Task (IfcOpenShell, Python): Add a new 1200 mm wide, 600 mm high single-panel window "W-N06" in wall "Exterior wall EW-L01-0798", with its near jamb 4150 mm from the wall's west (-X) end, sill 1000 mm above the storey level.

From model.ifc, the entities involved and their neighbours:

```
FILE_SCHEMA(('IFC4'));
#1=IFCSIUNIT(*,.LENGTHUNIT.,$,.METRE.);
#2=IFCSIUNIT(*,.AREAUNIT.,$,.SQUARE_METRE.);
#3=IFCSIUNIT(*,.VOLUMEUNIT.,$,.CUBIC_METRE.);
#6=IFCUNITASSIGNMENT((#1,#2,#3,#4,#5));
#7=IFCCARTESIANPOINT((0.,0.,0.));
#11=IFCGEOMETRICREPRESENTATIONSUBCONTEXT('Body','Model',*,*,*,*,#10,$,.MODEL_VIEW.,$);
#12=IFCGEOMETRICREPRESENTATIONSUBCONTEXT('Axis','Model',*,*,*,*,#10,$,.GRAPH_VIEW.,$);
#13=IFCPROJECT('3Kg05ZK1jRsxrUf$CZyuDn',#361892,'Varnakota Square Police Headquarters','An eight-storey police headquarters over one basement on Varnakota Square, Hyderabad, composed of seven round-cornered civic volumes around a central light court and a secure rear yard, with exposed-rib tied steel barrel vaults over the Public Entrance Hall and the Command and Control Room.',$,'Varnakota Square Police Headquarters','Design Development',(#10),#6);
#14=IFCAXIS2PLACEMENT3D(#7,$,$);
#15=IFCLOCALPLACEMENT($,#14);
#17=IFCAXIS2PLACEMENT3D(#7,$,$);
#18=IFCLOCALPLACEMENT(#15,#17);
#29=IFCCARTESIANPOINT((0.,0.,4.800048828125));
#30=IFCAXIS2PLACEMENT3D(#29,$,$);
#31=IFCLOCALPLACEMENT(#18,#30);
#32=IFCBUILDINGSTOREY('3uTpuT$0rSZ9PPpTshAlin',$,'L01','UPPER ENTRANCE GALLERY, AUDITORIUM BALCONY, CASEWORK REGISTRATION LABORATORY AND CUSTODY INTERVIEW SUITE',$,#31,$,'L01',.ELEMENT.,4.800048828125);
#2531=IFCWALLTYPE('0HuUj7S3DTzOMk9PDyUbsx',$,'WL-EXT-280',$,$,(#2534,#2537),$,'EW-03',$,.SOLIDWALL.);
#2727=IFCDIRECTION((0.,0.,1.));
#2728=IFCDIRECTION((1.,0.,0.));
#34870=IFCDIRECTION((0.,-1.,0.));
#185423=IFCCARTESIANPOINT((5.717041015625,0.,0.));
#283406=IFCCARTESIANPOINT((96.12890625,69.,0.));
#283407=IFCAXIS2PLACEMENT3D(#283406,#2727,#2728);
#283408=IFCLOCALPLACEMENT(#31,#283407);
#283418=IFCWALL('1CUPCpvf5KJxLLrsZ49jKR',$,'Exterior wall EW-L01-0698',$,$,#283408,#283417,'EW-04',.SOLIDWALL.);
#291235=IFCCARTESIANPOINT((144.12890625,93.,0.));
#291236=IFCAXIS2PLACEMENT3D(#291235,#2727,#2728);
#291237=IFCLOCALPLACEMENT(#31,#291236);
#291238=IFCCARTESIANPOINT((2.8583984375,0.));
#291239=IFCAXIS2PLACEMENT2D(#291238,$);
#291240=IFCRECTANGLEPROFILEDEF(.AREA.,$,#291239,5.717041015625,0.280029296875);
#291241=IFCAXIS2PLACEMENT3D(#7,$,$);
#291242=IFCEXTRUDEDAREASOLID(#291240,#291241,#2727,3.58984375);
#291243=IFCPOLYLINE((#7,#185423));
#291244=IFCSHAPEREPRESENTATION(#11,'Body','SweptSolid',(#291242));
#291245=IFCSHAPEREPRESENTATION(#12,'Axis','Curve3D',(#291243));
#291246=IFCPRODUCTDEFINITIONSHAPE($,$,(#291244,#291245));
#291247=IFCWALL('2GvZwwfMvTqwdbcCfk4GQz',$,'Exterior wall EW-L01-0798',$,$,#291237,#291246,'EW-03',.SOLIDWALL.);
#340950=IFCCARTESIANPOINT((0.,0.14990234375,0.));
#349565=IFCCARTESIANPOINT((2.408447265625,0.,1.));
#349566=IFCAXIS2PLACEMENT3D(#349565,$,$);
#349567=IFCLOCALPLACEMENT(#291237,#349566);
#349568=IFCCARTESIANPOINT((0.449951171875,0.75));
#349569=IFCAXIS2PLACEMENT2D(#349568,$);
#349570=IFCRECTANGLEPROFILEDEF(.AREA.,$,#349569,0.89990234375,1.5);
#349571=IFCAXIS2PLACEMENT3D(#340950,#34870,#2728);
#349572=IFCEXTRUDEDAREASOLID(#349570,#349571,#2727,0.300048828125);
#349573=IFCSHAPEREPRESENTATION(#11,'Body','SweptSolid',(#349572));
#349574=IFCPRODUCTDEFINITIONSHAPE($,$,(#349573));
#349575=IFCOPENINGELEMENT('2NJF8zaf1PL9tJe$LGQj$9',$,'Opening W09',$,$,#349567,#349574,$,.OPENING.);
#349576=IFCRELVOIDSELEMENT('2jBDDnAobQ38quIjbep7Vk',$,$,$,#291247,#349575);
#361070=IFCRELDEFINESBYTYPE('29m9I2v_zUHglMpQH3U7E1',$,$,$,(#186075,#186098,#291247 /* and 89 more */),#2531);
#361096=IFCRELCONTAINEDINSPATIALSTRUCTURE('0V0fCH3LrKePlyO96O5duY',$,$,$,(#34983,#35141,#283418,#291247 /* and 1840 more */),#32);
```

```python
import numpy as np
import ifcopenshell
import ifcopenshell.api.feature
import ifcopenshell.api.geometry
import ifcopenshell.api.root
import ifcopenshell.api.spatial
import ifcopenshell.geom
import ifcopenshell.util.element
import ifcopenshell.util.placement
import ifcopenshell.util.representation
import ifcopenshell.util.shape
import ifcopenshell.util.unit

model = ifcopenshell.open("model.ifc")
unit_scale = ifcopenshell.util.unit.calculate_unit_scale(model)
settings = ifcopenshell.geom.settings()


def volume(element):
    """Net volume in cubic metres, openings subtracted."""
    shape = ifcopenshell.geom.create_shape(settings, element)
    return ifcopenshell.util.shape.get_volume(shape.geometry)


wall = model.by_guid("2GvZwwfMvTqwdbcCfk4GQz")
storey = ifcopenshell.util.element.get_container(wall, ifc_class="IfcBuildingStorey")
context = ifcopenshell.util.representation.get_context(model, "Model", "Body", "MODEL_VIEW")
before = volume(wall)

width, height, from_end, sill = 1.2, 0.6, 4.15, 1  # metres

# The wall runs along its own X axis, and the end named is its -X end.
wall_shape = ifcopenshell.geom.create_shape(settings, wall)
x, y, z = ifcopenshell.util.shape.get_vertices(wall_shape.geometry).T
start = x.min() + from_end
face, thickness = float(y.min()), float(y.max() - y.min())
wall_matrix = ifcopenshell.util.placement.get_local_placement(wall.ObjectPlacement)
level = ifcopenshell.util.placement.get_local_placement(storey.ObjectPlacement)[2, 3]


def in_wall(x, y):
    """Placement at x, y metres in the wall's axes, at sill height."""
    matrix = wall_matrix.copy()
    matrix[:, 3] = wall_matrix @ np.array([x / unit_scale, y / unit_scale, 0.0, 1.0])
    matrix[2, 3] = level + sill / unit_scale
    return matrix


# Opening: a box that overshoots both wall faces by 50 mm.
opening = ifcopenshell.api.root.create_entity(model, ifc_class="IfcOpeningElement", predefined_type="OPENING")
box = ifcopenshell.api.geometry.add_wall_representation(
    model, context=context, length=width, height=height, thickness=thickness + 0.1
)
ifcopenshell.api.geometry.assign_representation(model, product=opening, representation=box)
ifcopenshell.api.geometry.edit_object_placement(model, product=opening, matrix=in_wall(start, face - 0.05), is_si=False)
ifcopenshell.api.feature.add_feature(model, feature=opening, element=wall)

window = ifcopenshell.api.root.create_entity(model, ifc_class="IfcWindow", name="W-N06", predefined_type="WINDOW")
window.OverallWidth, window.OverallHeight = width / unit_scale, height / unit_scale
window.PartitioningType = "SINGLE_PANEL"
body = ifcopenshell.api.geometry.add_window_representation(
    model,
    context=context,
    overall_width=window.OverallWidth,
    overall_height=window.OverallHeight,
    partition_type="SINGLE_PANEL",
)
ifcopenshell.api.geometry.assign_representation(model, product=window, representation=body)
ifcopenshell.api.spatial.assign_container(model, products=[window], relating_structure=storey)
ifcopenshell.api.feature.add_filling(model, opening=opening, element=window)

# Centre the window in the wall's thickness.
ifcopenshell.api.geometry.edit_object_placement(model, product=window, matrix=in_wall(start, face), is_si=False)
window_shape = ifcopenshell.geom.create_shape(settings, window)
depth = ifcopenshell.util.shape.get_vertices(window_shape.geometry)[:, 1]
offset = face + thickness / 2 - (depth.min() + depth.max()) / 2
ifcopenshell.api.geometry.edit_object_placement(model, product=window, matrix=in_wall(start, offset), is_si=False)

after = volume(wall)

print(f"wall volume {before:.3f} -> {after:.3f} m3")

model.write("model_updated.ifc")
```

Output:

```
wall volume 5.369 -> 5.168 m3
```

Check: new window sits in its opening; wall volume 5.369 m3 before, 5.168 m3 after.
